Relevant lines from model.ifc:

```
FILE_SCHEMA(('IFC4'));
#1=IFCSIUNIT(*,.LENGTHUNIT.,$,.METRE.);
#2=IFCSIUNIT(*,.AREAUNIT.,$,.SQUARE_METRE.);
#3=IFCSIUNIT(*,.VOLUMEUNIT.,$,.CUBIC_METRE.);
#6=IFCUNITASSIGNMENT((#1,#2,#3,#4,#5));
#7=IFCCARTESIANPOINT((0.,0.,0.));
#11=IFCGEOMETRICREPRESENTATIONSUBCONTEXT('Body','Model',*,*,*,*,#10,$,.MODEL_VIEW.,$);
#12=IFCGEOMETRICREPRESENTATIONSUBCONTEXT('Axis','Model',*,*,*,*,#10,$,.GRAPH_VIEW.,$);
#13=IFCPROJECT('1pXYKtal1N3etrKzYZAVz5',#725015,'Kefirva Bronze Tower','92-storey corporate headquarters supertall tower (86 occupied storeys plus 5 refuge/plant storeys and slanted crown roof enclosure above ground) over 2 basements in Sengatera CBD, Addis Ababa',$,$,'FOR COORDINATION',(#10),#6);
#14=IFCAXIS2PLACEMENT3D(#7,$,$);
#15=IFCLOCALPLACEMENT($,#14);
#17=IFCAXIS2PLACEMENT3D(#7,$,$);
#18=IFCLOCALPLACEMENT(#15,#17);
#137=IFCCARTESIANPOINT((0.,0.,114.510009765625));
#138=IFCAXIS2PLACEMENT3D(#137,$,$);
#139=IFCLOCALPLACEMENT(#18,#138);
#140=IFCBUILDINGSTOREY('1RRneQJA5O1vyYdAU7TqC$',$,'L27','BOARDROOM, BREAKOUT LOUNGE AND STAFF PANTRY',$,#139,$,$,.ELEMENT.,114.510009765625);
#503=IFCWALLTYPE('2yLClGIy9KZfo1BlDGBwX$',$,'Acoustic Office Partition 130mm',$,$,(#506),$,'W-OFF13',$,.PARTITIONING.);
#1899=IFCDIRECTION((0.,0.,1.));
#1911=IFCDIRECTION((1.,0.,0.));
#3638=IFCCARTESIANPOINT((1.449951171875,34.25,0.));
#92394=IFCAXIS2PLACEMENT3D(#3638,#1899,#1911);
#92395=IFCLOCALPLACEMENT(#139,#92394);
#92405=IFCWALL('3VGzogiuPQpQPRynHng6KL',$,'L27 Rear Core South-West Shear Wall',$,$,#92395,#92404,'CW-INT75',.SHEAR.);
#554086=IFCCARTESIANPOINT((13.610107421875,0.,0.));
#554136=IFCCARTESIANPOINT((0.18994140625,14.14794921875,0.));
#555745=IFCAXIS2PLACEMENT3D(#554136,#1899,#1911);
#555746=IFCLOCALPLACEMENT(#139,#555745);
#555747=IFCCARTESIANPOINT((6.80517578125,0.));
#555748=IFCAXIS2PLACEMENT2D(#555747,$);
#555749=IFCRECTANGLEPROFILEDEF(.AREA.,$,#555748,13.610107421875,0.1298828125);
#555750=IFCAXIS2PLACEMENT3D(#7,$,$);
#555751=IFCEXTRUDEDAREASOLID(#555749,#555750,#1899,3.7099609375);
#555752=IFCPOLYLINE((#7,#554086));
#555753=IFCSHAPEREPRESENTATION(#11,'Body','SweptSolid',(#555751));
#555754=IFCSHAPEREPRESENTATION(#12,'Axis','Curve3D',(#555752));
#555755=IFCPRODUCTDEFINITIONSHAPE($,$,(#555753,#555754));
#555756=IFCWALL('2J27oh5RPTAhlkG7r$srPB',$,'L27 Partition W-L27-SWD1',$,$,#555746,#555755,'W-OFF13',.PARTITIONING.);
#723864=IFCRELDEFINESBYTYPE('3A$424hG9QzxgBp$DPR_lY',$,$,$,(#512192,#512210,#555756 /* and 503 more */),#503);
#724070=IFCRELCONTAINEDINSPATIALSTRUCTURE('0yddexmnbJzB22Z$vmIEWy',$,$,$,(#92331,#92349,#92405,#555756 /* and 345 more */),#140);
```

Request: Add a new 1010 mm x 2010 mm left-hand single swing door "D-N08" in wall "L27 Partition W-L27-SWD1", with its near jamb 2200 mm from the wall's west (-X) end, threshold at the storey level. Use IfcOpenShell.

```python
import numpy as np
import ifcopenshell
import ifcopenshell.api.feature
import ifcopenshell.api.geometry
import ifcopenshell.api.root
import ifcopenshell.api.spatial
import ifcopenshell.geom
import ifcopenshell.util.element
import ifcopenshell.util.placement
import ifcopenshell.util.representation
import ifcopenshell.util.shape
import ifcopenshell.util.unit

model = ifcopenshell.open("model.ifc")
unit_scale = ifcopenshell.util.unit.calculate_unit_scale(model)
settings = ifcopenshell.geom.settings()


def volume(element):
    """Net volume in cubic metres, openings subtracted."""
    shape = ifcopenshell.geom.create_shape(settings, element)
    return ifcopenshell.util.shape.get_volume(shape.geometry)


wall = model.by_guid("2J27oh5RPTAhlkG7r$srPB")
storey = ifcopenshell.util.element.get_container(wall, ifc_class="IfcBuildingStorey")
context = ifcopenshell.util.representation.get_context(model, "Model", "Body", "MODEL_VIEW")
before = volume(wall)

width, height, from_end, sill = 1.01, 2.01, 2.2, 0.0  # metres

# The wall runs along its own X axis, and the end named is its -X end.
wall_shape = ifcopenshell.geom.create_shape(settings, wall)
x, y, z = ifcopenshell.util.shape.get_vertices(wall_shape.geometry).T
start = x.min() + from_end
face, thickness = float(y.min()), float(y.max() - y.min())
wall_matrix = ifcopenshell.util.placement.get_local_placement(wall.ObjectPlacement)
level = ifcopenshell.util.placement.get_local_placement(storey.ObjectPlacement)[2, 3]


def in_wall(x, y):
    """Placement at x, y metres in the wall's axes, at sill height."""
    matrix = wall_matrix.copy()
    matrix[:, 3] = wall_matrix @ np.array([x / unit_scale, y / unit_scale, 0.0, 1.0])
    matrix[2, 3] = level + sill / unit_scale
    return matrix


# Opening: a box that overshoots both wall faces by 50 mm.
opening = ifcopenshell.api.root.create_entity(model, ifc_class="IfcOpeningElement", predefined_type="OPENING")
box = ifcopenshell.api.geometry.add_wall_representation(
    model, context=context, length=width, height=height, thickness=thickness + 0.1
)
ifcopenshell.api.geometry.assign_representation(model, product=opening, representation=box)
ifcopenshell.api.geometry.edit_object_placement(model, product=opening, matrix=in_wall(start, face - 0.05), is_si=False)
ifcopenshell.api.feature.add_feature(model, feature=opening, element=wall)

door = ifcopenshell.api.root.create_entity(model, ifc_class="IfcDoor", name="D-N08", predefined_type="DOOR")
door.OverallWidth, door.OverallHeight = width / unit_scale, height / unit_scale
door.OperationType = "SINGLE_SWING_LEFT"
body = ifcopenshell.api.geometry.add_door_representation(
    model,
    context=context,
    overall_width=door.OverallWidth,
    overall_height=door.OverallHeight,
    operation_type="SINGLE_SWING_LEFT",
    lining_properties={"LiningDepth": thickness / unit_scale, "ThresholdDepth": thickness / unit_scale},
)
ifcopenshell.api.geometry.assign_representation(model, product=door, representation=body)
ifcopenshell.api.spatial.assign_container(model, products=[door], relating_structure=storey)
ifcopenshell.api.feature.add_filling(model, opening=opening, element=door)

# The lining spans the wall, so the door starts at the wall face.
ifcopenshell.api.geometry.edit_object_placement(model, product=door, matrix=in_wall(start, face), is_si=False)

after = volume(wall)

print(f"wall volume {before:.3f} -> {after:.3f} m3")

model.write("model_v2.ifc")
```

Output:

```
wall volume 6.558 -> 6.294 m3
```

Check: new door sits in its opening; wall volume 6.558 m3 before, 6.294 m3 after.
